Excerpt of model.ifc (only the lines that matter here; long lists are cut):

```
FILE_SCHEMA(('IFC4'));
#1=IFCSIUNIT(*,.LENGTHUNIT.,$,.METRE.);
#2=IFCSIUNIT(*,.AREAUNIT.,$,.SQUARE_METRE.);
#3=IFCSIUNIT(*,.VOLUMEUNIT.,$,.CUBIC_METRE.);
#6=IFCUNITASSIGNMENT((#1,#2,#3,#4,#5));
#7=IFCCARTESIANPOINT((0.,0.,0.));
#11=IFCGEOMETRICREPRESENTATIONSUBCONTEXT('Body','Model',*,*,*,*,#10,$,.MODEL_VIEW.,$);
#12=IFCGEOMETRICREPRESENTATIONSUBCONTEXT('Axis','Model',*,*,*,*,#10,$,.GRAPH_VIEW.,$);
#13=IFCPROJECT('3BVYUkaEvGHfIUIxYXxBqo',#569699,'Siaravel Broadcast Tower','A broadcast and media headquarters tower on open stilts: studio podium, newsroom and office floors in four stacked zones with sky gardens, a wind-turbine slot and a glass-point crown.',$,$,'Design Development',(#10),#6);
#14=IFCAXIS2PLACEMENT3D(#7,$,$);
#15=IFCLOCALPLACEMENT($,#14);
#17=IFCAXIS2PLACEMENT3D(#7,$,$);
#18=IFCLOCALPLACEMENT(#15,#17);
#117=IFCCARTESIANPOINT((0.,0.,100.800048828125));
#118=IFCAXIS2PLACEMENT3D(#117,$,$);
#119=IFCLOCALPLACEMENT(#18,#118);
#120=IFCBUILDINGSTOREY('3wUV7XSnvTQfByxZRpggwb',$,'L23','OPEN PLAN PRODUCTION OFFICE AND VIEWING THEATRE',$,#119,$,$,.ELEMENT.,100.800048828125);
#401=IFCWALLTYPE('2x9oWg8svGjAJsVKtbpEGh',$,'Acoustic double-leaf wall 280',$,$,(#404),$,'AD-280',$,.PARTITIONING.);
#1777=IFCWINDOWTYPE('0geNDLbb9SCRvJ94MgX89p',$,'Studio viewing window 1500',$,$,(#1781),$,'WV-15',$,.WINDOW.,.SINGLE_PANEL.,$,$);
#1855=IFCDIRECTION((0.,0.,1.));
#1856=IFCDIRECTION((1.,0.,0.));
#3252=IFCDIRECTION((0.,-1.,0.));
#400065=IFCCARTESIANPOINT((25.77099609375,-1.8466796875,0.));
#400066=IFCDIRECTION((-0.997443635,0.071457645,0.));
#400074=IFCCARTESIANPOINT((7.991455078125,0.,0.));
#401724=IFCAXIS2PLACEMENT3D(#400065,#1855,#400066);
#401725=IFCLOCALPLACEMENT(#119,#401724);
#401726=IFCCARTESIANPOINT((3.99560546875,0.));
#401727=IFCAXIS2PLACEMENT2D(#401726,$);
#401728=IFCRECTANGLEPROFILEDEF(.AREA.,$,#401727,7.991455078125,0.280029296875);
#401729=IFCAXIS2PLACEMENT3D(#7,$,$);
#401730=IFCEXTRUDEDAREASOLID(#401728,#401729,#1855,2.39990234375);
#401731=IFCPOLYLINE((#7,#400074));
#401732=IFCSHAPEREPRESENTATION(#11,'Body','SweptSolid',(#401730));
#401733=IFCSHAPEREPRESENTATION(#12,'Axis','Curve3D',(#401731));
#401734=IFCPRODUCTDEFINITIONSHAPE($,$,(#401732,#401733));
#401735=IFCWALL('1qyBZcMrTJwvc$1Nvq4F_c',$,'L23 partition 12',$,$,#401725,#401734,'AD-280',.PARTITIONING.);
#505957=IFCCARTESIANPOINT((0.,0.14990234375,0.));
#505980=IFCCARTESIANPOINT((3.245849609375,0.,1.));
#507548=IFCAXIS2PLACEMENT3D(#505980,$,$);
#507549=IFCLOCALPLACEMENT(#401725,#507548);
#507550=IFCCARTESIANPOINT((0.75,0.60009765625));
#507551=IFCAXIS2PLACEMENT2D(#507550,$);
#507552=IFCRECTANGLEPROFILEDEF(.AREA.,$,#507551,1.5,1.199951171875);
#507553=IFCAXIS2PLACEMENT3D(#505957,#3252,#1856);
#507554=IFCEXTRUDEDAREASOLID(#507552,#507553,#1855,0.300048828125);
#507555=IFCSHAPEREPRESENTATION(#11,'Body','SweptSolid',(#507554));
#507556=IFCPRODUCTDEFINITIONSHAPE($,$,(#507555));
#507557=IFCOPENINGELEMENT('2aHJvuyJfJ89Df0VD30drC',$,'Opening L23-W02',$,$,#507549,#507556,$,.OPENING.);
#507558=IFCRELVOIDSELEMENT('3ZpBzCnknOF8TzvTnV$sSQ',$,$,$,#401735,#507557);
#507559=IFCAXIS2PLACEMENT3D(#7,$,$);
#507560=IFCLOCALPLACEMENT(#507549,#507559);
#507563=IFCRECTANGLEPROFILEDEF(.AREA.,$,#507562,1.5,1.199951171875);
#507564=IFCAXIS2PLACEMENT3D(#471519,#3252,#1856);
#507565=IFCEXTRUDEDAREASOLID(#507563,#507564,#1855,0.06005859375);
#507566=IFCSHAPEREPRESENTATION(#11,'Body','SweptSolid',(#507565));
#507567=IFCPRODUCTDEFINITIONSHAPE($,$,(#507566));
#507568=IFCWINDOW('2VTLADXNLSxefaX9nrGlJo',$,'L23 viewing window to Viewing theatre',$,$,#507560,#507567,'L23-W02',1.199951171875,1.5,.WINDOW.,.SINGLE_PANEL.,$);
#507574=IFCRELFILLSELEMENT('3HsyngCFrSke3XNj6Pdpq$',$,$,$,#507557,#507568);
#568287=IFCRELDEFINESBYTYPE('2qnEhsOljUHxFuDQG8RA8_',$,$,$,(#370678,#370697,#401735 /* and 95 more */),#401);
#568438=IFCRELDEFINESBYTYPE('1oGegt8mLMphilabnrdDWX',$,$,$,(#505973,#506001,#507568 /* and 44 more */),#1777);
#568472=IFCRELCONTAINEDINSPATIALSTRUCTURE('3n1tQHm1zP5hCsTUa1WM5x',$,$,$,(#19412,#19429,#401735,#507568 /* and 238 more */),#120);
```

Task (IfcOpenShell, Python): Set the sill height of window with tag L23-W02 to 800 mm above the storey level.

```python
import numpy as np
import ifcopenshell
import ifcopenshell.api.geometry
import ifcopenshell.geom
import ifcopenshell.util.element
import ifcopenshell.util.placement
import ifcopenshell.util.shape
import ifcopenshell.util.unit

model = ifcopenshell.open("model.ifc")
unit_scale = ifcopenshell.util.unit.calculate_unit_scale(model)

window = model.by_guid("2VTLADXNLSxefaX9nrGlJo")
opening = window.FillsVoids[0].RelatingOpeningElement
storey = ifcopenshell.util.element.get_container(window, ifc_class="IfcBuildingStorey")
level = ifcopenshell.util.placement.get_local_placement(storey.ObjectPlacement)[2, 3]

# The opening's origin need not be at the sill, so measure its lowest point.
shape = ifcopenshell.geom.create_shape(ifcopenshell.geom.settings(), opening)
bottom = ifcopenshell.util.shape.get_shape_bottom_elevation(shape, shape.geometry) / unit_scale
dz = level + 0.8 - bottom

shift = np.array([0.0, 0.0, dz])
# The window is placed relative to its opening, so it follows when the opening moves.
matrix = ifcopenshell.util.placement.get_local_placement(opening.ObjectPlacement)
matrix[:3, 3] += shift
ifcopenshell.api.geometry.edit_object_placement(
    model, product=opening, matrix=matrix, is_si=False, should_transform_children=True
)

print(f"moved by {dz * unit_scale:+.3f} m")

model.write("model-out.ifc")
```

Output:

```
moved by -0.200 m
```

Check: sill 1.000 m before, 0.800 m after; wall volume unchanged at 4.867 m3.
